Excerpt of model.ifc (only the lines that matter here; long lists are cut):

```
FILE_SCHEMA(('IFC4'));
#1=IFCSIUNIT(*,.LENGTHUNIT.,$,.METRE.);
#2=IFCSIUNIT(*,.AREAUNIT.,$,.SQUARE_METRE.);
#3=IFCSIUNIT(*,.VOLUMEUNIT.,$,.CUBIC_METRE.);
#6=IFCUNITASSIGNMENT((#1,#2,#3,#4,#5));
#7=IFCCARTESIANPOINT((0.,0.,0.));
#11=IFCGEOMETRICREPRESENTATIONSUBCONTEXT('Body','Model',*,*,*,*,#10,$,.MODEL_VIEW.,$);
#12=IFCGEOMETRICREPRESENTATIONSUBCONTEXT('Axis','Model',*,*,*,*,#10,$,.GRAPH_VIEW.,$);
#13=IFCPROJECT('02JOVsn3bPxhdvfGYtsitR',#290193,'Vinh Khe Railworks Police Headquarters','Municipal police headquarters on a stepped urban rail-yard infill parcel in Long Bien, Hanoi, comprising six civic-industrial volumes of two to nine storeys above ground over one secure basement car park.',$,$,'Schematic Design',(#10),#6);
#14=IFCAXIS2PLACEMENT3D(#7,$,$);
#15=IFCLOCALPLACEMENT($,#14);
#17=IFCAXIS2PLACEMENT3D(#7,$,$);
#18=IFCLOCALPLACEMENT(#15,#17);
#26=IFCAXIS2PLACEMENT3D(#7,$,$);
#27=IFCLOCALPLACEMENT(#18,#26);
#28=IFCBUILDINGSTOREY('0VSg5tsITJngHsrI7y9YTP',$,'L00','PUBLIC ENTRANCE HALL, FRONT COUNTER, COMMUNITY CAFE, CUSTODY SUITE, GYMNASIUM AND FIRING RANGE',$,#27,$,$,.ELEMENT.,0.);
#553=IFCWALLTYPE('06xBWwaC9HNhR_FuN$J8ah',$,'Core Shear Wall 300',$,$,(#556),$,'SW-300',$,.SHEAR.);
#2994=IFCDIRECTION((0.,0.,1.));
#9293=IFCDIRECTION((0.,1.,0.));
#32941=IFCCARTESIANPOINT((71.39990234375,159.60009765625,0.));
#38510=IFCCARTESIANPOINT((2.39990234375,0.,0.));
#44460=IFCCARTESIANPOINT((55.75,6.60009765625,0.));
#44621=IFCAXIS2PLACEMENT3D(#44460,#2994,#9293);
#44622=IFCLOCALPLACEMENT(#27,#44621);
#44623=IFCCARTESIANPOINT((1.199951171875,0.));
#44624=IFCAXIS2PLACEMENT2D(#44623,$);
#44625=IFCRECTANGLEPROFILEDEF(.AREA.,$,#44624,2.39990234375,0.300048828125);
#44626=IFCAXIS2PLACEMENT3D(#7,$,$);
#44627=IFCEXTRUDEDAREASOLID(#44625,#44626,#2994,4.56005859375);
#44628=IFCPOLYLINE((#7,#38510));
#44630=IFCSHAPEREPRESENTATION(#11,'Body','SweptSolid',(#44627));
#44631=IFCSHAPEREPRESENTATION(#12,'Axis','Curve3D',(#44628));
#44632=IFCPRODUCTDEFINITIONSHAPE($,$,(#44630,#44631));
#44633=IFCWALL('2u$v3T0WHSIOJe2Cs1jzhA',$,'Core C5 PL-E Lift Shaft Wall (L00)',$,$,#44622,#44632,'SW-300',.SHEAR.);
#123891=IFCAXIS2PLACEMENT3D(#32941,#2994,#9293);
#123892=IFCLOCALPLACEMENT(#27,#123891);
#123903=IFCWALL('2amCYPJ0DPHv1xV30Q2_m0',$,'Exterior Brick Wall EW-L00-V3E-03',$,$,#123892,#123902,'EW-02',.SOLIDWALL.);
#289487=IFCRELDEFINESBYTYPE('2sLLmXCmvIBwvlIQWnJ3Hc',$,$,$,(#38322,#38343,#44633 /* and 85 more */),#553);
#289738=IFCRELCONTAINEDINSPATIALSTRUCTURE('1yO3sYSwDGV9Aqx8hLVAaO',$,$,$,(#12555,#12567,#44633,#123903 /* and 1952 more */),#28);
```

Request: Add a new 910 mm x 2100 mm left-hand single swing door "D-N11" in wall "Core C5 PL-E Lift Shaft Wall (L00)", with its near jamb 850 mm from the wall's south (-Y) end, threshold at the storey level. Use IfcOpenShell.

```python
import numpy as np
import ifcopenshell
import ifcopenshell.api.feature
import ifcopenshell.api.geometry
import ifcopenshell.api.root
import ifcopenshell.api.spatial
import ifcopenshell.geom
import ifcopenshell.util.element
import ifcopenshell.util.placement
import ifcopenshell.util.representation
import ifcopenshell.util.shape
import ifcopenshell.util.unit

model = ifcopenshell.open("model.ifc")
unit_scale = ifcopenshell.util.unit.calculate_unit_scale(model)
settings = ifcopenshell.geom.settings()


def volume(element):
    """Net volume in cubic metres, openings subtracted."""
    shape = ifcopenshell.geom.create_shape(settings, element)
    return ifcopenshell.util.shape.get_volume(shape.geometry)


wall = model.by_id(44633)
storey = ifcopenshell.util.element.get_container(wall, ifc_class="IfcBuildingStorey")
context = ifcopenshell.util.representation.get_context(model, "Model", "Body", "MODEL_VIEW")
before = volume(wall)

width, height, from_end, sill = 0.91, 2.1, 0.85, 0.0  # metres

# The wall runs along its own X axis, and the end named is its -X end.
wall_shape = ifcopenshell.geom.create_shape(settings, wall)
x, y, z = ifcopenshell.util.shape.get_vertices(wall_shape.geometry).T
start = x.min() + from_end
face, thickness = float(y.min()), float(y.max() - y.min())
wall_matrix = ifcopenshell.util.placement.get_local_placement(wall.ObjectPlacement)
level = ifcopenshell.util.placement.get_local_placement(storey.ObjectPlacement)[2, 3]


def in_wall(x, y):
    """Placement at x, y metres in the wall's axes, at sill height."""
    matrix = wall_matrix.copy()
    matrix[:, 3] = wall_matrix @ np.array([x / unit_scale, y / unit_scale, 0.0, 1.0])
    matrix[2, 3] = level + sill / unit_scale
    return matrix


# Opening: a box that overshoots both wall faces by 50 mm.
opening = ifcopenshell.api.root.create_entity(model, ifc_class="IfcOpeningElement", predefined_type="OPENING")
box = ifcopenshell.api.geometry.add_wall_representation(
    model, context=context, length=width, height=height, thickness=thickness + 0.1
)
ifcopenshell.api.geometry.assign_representation(model, product=opening, representation=box)
ifcopenshell.api.geometry.edit_object_placement(model, product=opening, matrix=in_wall(start, face - 0.05), is_si=False)
ifcopenshell.api.feature.add_feature(model, feature=opening, element=wall)

door = ifcopenshell.api.root.create_entity(model, ifc_class="IfcDoor", name="D-N11", predefined_type="DOOR")
door.OverallWidth, door.OverallHeight = width / unit_scale, height / unit_scale
door.OperationType = "SINGLE_SWING_LEFT"
body = ifcopenshell.api.geometry.add_door_representation(
    model,
    context=context,
    overall_width=door.OverallWidth,
    overall_height=door.OverallHeight,
    operation_type="SINGLE_SWING_LEFT",
    lining_properties={"LiningDepth": thickness / unit_scale, "ThresholdDepth": thickness / unit_scale},
)
ifcopenshell.api.geometry.assign_representation(model, product=door, representation=body)
ifcopenshell.api.spatial.assign_container(model, products=[door], relating_structure=storey)
ifcopenshell.api.feature.add_filling(model, opening=opening, element=door)

# The lining spans the wall, so the door starts at the wall face.
ifcopenshell.api.geometry.edit_object_placement(model, product=door, matrix=in_wall(start, face), is_si=False)

after = volume(wall)

print(f"wall volume {before:.3f} -> {after:.3f} m3")

model.write("model_edited.ifc")
```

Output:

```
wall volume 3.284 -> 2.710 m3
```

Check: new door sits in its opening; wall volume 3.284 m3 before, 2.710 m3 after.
